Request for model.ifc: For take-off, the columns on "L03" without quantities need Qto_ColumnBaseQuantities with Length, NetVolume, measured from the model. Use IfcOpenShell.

First a look at what the model holds.

```python
import ifcopenshell
import ifcopenshell.util.element
import ifcopenshell.util.unit

model = ifcopenshell.open("model.ifc")
print(model.schema)
for unit_type in ("LENGTHUNIT", "AREAUNIT", "VOLUMEUNIT"):
    print(unit_type, ifcopenshell.util.unit.calculate_unit_scale(model, unit_type))
storey = next(s for s in model.by_type("IfcBuildingStorey") if s.Name == "L03")
columns = [e for e in ifcopenshell.util.element.get_decomposition(storey) if e.is_a("IfcColumn")]
for e in sorted(columns, key=lambda e: e.id()):
    print(e.id(), e.is_a(), e.Name, list(ifcopenshell.util.element.get_psets(e, qtos_only=True)), sep=" | ")
```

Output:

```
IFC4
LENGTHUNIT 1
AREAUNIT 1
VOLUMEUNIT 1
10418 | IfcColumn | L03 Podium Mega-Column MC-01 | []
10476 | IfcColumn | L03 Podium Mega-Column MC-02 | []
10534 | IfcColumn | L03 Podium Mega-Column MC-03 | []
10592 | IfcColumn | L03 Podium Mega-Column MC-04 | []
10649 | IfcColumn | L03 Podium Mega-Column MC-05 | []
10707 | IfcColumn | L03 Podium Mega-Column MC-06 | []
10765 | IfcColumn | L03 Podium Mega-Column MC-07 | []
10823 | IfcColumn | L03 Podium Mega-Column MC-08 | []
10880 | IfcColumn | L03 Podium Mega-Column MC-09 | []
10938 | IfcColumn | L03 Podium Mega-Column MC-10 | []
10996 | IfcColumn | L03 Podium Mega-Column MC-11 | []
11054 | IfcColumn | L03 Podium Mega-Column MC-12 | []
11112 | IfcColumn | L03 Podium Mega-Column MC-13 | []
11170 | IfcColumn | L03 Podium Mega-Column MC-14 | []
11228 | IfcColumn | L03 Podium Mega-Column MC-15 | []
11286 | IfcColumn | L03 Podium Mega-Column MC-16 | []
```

```python
import ifcopenshell
import ifcopenshell.api.pset
import ifcopenshell.geom
import ifcopenshell.util.element
import ifcopenshell.util.shape
import ifcopenshell.util.unit

model = ifcopenshell.open("model.ifc")
unit_scale = ifcopenshell.util.unit.calculate_unit_scale(model)
volume_scale = ifcopenshell.util.unit.calculate_unit_scale(model, "VOLUMEUNIT")
settings = ifcopenshell.geom.settings()

storey = next(s for s in model.by_type("IfcBuildingStorey") if s.Name == "L03")
columns = [e for e in ifcopenshell.util.element.get_decomposition(storey) if e.is_a("IfcColumn")]

for e in sorted(columns, key=lambda e: e.id()):
    if ifcopenshell.util.element.get_psets(e, qtos_only=True, should_inherit=False):
        continue
    # Geometry comes back in metres, in the element's own axes.
    shape = ifcopenshell.geom.create_shape(settings, e)
    values = {
        "Length": ifcopenshell.util.shape.get_z(shape.geometry) / unit_scale,
        "NetVolume": ifcopenshell.util.shape.get_volume(shape.geometry) / volume_scale,
    }
    qto = ifcopenshell.api.pset.add_qto(model, product=e, name="Qto_ColumnBaseQuantities")
    ifcopenshell.api.pset.edit_qto(model, qto=qto, properties=values)
    print(e.id(), {k: round(v, 3) for k, v in values.items()})

model.write("model_v2.ifc")
```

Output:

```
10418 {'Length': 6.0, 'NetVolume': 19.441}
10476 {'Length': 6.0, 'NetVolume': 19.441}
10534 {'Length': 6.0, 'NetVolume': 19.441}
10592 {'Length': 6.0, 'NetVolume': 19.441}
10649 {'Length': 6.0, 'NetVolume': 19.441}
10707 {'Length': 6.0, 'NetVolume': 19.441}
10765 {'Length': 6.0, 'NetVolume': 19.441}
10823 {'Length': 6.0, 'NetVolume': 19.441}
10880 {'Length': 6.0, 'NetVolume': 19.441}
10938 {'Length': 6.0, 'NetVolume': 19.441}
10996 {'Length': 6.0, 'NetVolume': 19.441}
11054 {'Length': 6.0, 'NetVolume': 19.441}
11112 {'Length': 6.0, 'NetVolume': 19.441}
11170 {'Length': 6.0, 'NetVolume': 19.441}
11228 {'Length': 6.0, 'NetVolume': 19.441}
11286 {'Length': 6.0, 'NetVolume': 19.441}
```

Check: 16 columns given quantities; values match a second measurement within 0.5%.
